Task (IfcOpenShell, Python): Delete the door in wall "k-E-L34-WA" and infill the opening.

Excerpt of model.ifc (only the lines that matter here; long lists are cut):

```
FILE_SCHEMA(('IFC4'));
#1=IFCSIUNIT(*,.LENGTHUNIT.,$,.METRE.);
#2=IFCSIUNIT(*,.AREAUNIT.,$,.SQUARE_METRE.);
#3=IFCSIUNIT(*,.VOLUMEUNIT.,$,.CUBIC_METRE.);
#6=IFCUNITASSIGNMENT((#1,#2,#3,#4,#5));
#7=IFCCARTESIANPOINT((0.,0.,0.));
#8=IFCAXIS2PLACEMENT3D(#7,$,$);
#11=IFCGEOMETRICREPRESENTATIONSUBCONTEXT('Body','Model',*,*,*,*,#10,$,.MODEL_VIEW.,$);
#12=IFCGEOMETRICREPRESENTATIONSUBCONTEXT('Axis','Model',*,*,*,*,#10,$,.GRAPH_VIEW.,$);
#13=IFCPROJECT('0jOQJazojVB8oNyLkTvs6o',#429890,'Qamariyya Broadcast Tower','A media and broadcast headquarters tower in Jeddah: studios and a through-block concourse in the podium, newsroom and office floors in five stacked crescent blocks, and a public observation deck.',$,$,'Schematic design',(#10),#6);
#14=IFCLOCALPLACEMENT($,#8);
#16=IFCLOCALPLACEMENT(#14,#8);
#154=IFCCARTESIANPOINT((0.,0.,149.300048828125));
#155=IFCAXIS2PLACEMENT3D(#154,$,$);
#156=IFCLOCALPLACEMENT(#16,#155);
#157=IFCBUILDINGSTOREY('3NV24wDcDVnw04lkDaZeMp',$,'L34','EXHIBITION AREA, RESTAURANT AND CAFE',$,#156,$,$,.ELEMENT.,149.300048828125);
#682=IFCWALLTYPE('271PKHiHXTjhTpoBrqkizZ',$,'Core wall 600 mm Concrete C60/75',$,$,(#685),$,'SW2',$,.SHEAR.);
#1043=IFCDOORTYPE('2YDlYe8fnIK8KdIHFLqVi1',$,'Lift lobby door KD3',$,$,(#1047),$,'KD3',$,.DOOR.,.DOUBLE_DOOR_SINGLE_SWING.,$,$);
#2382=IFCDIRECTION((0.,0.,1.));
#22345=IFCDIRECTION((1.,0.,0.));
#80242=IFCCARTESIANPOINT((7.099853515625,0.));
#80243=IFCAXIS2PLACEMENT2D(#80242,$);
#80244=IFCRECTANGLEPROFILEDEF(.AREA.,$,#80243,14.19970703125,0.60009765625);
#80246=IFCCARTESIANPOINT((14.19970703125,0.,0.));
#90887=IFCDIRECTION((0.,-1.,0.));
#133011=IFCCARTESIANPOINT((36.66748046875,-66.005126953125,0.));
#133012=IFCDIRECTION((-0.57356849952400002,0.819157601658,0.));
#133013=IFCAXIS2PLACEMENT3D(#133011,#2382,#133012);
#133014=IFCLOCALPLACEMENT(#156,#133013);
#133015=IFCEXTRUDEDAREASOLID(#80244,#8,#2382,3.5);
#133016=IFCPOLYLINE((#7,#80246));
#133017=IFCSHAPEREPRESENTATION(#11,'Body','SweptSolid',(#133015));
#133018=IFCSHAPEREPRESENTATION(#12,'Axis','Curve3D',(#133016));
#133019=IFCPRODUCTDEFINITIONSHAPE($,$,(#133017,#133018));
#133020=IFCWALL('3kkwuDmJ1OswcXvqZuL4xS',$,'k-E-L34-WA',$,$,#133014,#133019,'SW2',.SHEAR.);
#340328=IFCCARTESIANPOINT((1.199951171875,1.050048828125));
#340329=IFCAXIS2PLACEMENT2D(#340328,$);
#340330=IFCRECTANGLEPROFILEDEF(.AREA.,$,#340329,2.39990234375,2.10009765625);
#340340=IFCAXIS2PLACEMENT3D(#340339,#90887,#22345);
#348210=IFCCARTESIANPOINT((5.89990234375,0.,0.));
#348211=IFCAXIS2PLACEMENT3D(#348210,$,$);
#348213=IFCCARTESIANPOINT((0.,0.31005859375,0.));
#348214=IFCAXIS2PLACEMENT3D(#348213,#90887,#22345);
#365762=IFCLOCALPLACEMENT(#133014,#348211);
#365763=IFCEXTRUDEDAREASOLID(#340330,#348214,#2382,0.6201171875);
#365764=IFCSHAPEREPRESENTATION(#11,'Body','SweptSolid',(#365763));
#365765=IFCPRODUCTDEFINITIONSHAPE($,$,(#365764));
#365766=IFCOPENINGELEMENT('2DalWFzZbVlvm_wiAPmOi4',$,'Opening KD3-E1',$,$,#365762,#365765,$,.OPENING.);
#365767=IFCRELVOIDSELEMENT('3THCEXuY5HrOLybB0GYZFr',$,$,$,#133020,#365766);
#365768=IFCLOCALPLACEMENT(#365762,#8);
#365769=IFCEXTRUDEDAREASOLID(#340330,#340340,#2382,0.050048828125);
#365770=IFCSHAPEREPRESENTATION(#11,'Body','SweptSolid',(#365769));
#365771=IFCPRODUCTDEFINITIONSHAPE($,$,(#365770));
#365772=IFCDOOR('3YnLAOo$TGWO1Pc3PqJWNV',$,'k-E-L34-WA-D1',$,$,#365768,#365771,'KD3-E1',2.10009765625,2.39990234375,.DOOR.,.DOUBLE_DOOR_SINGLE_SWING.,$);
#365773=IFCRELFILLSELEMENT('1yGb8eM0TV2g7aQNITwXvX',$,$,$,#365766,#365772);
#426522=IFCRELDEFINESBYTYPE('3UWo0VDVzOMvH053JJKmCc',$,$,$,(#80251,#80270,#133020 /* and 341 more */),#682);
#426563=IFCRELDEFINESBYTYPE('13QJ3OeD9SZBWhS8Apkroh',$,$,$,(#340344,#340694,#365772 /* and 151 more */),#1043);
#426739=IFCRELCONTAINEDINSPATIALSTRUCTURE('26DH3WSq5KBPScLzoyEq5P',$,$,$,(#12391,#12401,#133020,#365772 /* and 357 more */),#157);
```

```python
import ifcopenshell
import ifcopenshell.api.feature
import ifcopenshell.api.root
import ifcopenshell.geom
import ifcopenshell.util.shape

model = ifcopenshell.open("model.ifc")
settings = ifcopenshell.geom.settings()


def volume(element):
    """Net volume in cubic metres, openings subtracted."""
    shape = ifcopenshell.geom.create_shape(settings, element)
    return ifcopenshell.util.shape.get_volume(shape.geometry)


door = model.by_guid("3YnLAOo$TGWO1Pc3PqJWNV")
opening = door.FillsVoids[0].RelatingOpeningElement
wall = opening.VoidsElements[0].RelatingBuildingElement
before = volume(wall)

ifcopenshell.api.root.remove_product(model, product=door)
ifcopenshell.api.feature.remove_feature(model, feature=opening)

after = volume(wall)

print(f"wall volume {before:.3f} -> {after:.3f} m3")

model.write("model_edited.ifc")
```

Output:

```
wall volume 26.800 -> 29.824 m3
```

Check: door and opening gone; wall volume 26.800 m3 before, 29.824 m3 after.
